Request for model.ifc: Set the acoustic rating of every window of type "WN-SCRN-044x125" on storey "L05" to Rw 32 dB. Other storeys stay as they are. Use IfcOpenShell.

First a look at what the model holds.

```python
import ifcopenshell
import ifcopenshell.util.element

model = ifcopenshell.open("model.ifc")
print(model.schema)
storey = next(s for s in model.by_type("IfcBuildingStorey") if s.Name == "L05")
windows = [e for e in ifcopenshell.util.element.get_decomposition(storey) if e.is_a("IfcWindow")]
seen = {}
for e in windows:
    element_type = ifcopenshell.util.element.get_type(e)
    key = (element_type.Name if element_type != e and element_type else None, ifcopenshell.util.element.get_pset(e, "Pset_WindowCommon", "AcousticRating"))
    seen[key] = seen.get(key, 0) + 1
for (name, value), count in sorted(seen.items(), key=str):
    print(count, "x", name, "|", value)
```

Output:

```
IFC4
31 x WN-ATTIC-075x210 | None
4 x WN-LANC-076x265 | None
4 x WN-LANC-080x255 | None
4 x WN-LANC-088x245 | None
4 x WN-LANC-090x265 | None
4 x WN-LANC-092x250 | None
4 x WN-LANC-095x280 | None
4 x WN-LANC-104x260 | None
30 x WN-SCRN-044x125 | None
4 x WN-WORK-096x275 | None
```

```python
import ifcopenshell
import ifcopenshell.api.pset
import ifcopenshell.util.element

model = ifcopenshell.open("model.ifc")

storey = next(s for s in model.by_type("IfcBuildingStorey") if s.Name == "L05")
windows = [e for e in ifcopenshell.util.element.get_decomposition(storey) if e.is_a("IfcWindow")]

count = 0
for e in windows:
    element_type = ifcopenshell.util.element.get_type(e)
    if element_type in (None, e) or element_type.Name != "WN-SCRN-044x125":
        continue
    # add_pset returns the element's existing set when there is one.
    pset = ifcopenshell.api.pset.add_pset(model, product=e, name="Pset_WindowCommon")
    ifcopenshell.api.pset.edit_pset(model, pset=pset, properties={"AcousticRating": "Rw 32 dB"})
    count += 1

print(count, "windows updated")

model.write("model-out.ifc")
```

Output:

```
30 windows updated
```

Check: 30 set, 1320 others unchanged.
